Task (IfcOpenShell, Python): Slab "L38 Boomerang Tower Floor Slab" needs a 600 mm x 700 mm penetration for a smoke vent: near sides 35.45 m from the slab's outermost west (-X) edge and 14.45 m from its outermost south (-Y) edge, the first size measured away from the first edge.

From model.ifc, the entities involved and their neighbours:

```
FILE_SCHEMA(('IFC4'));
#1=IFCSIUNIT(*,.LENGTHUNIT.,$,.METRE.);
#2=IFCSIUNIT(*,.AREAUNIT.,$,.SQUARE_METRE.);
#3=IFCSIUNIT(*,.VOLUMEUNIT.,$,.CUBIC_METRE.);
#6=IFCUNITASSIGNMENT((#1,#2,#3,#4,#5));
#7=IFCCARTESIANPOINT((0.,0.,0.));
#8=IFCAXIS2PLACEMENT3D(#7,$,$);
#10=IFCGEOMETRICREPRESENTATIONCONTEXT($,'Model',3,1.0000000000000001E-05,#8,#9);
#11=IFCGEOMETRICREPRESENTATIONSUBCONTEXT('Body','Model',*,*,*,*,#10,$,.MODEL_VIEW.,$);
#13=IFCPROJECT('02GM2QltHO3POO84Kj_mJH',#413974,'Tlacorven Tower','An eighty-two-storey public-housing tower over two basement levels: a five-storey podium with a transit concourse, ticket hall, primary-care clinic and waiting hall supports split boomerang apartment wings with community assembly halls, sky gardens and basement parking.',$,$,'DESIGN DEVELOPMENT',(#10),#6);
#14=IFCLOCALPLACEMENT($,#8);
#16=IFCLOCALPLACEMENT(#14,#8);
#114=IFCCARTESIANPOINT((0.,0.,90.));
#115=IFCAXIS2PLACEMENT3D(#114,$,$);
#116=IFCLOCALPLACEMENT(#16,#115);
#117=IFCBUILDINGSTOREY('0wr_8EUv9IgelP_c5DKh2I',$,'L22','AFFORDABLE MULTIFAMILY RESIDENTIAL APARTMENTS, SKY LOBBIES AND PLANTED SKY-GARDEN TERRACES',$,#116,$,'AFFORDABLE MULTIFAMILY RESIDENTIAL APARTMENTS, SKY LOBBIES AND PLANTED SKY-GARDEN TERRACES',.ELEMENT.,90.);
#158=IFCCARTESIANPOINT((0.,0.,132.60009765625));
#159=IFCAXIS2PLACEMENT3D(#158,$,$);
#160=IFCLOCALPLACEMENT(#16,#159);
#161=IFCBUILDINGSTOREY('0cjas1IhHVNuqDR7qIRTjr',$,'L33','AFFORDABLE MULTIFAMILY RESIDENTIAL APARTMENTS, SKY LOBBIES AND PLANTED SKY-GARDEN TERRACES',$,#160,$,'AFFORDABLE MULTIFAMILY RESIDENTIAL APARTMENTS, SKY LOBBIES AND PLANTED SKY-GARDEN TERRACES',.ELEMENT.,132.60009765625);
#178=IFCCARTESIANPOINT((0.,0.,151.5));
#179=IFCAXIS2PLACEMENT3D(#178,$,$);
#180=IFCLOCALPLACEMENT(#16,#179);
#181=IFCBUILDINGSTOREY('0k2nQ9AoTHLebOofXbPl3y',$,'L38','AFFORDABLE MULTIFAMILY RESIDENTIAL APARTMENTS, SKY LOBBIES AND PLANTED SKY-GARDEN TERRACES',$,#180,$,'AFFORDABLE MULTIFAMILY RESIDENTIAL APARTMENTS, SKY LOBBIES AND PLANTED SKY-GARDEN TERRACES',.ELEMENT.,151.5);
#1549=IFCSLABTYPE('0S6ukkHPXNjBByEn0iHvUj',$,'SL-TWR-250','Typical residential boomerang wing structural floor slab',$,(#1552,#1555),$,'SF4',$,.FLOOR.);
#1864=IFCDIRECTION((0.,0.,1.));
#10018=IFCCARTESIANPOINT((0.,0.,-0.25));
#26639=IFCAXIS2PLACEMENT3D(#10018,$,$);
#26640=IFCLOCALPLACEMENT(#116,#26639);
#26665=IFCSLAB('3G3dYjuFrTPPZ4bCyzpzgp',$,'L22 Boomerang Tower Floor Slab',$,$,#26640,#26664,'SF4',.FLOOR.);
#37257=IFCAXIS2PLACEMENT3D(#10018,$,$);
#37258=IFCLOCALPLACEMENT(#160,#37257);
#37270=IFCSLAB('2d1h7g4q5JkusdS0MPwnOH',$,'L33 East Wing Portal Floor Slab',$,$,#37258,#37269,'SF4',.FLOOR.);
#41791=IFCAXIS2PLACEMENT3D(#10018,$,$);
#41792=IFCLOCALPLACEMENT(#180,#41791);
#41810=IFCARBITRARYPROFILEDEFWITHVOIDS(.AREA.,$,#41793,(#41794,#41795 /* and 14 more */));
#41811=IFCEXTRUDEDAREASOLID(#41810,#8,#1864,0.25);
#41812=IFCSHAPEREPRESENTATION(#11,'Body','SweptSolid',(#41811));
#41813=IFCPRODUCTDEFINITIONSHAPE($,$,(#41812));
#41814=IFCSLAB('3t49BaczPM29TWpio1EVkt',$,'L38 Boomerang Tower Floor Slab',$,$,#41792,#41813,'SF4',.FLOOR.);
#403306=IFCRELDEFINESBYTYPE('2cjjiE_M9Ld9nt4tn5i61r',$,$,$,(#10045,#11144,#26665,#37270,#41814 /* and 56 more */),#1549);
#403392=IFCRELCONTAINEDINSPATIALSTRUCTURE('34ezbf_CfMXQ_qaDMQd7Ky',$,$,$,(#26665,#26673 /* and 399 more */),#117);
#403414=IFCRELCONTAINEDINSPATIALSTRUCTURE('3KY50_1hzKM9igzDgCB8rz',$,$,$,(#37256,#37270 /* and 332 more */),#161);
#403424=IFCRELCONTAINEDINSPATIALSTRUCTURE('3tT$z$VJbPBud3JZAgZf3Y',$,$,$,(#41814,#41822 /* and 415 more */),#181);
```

```python
import numpy as np
import ifcopenshell
import ifcopenshell.api.feature
import ifcopenshell.api.geometry
import ifcopenshell.api.root
import ifcopenshell.geom
import ifcopenshell.util.placement
import ifcopenshell.util.representation
import ifcopenshell.util.shape
import ifcopenshell.util.unit

model = ifcopenshell.open("model.ifc")
unit_scale = ifcopenshell.util.unit.calculate_unit_scale(model)
settings = ifcopenshell.geom.settings()


def volume(element):
    """Net volume in cubic metres, openings subtracted."""
    shape = ifcopenshell.geom.create_shape(settings, element)
    return ifcopenshell.util.shape.get_volume(shape.geometry)


slab = model.by_guid("3t49BaczPM29TWpio1EVkt")
before = volume(slab)

# Extent in the slab's own axes, in metres. The edges named are its -X and -Y sides.
slab_shape = ifcopenshell.geom.create_shape(settings, slab)
vertices = ifcopenshell.util.shape.get_vertices(slab_shape.geometry)
x_min, y_min, bottom = vertices.min(axis=0)
top = vertices[:, 2].max()

opening = ifcopenshell.api.root.create_entity(model, ifc_class="IfcOpeningElement", name="Smoke vent opening", predefined_type="OPENING")
context = ifcopenshell.util.representation.get_context(model, "Model", "Body", "MODEL_VIEW")
width, depth = 0.6, 0.7
outline = [(0.0, 0.0), (width, 0.0), (width, depth), (0.0, depth), (0.0, 0.0)]
# Overshoot both faces by 50 mm so the cut is clean.
shape = ifcopenshell.api.geometry.add_slab_representation(
    model, context=context, depth=top - bottom + 0.1, polyline=outline
)
ifcopenshell.api.geometry.assign_representation(model, product=opening, representation=shape)

matrix = ifcopenshell.util.placement.get_local_placement(slab.ObjectPlacement)
matrix[:, 3] = matrix @ np.append(np.array([x_min + 35.45, y_min + 14.45, bottom - 0.05]) / unit_scale, 1.0)
ifcopenshell.api.geometry.edit_object_placement(model, product=opening, matrix=matrix, is_si=False)
ifcopenshell.api.feature.add_feature(model, feature=opening, element=slab)

after = volume(slab)

print(f"slab volume {before:.3f} -> {after:.3f} m3")

model.write("model_updated.ifc")
```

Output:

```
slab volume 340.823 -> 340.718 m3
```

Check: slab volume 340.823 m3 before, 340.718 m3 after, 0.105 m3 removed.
